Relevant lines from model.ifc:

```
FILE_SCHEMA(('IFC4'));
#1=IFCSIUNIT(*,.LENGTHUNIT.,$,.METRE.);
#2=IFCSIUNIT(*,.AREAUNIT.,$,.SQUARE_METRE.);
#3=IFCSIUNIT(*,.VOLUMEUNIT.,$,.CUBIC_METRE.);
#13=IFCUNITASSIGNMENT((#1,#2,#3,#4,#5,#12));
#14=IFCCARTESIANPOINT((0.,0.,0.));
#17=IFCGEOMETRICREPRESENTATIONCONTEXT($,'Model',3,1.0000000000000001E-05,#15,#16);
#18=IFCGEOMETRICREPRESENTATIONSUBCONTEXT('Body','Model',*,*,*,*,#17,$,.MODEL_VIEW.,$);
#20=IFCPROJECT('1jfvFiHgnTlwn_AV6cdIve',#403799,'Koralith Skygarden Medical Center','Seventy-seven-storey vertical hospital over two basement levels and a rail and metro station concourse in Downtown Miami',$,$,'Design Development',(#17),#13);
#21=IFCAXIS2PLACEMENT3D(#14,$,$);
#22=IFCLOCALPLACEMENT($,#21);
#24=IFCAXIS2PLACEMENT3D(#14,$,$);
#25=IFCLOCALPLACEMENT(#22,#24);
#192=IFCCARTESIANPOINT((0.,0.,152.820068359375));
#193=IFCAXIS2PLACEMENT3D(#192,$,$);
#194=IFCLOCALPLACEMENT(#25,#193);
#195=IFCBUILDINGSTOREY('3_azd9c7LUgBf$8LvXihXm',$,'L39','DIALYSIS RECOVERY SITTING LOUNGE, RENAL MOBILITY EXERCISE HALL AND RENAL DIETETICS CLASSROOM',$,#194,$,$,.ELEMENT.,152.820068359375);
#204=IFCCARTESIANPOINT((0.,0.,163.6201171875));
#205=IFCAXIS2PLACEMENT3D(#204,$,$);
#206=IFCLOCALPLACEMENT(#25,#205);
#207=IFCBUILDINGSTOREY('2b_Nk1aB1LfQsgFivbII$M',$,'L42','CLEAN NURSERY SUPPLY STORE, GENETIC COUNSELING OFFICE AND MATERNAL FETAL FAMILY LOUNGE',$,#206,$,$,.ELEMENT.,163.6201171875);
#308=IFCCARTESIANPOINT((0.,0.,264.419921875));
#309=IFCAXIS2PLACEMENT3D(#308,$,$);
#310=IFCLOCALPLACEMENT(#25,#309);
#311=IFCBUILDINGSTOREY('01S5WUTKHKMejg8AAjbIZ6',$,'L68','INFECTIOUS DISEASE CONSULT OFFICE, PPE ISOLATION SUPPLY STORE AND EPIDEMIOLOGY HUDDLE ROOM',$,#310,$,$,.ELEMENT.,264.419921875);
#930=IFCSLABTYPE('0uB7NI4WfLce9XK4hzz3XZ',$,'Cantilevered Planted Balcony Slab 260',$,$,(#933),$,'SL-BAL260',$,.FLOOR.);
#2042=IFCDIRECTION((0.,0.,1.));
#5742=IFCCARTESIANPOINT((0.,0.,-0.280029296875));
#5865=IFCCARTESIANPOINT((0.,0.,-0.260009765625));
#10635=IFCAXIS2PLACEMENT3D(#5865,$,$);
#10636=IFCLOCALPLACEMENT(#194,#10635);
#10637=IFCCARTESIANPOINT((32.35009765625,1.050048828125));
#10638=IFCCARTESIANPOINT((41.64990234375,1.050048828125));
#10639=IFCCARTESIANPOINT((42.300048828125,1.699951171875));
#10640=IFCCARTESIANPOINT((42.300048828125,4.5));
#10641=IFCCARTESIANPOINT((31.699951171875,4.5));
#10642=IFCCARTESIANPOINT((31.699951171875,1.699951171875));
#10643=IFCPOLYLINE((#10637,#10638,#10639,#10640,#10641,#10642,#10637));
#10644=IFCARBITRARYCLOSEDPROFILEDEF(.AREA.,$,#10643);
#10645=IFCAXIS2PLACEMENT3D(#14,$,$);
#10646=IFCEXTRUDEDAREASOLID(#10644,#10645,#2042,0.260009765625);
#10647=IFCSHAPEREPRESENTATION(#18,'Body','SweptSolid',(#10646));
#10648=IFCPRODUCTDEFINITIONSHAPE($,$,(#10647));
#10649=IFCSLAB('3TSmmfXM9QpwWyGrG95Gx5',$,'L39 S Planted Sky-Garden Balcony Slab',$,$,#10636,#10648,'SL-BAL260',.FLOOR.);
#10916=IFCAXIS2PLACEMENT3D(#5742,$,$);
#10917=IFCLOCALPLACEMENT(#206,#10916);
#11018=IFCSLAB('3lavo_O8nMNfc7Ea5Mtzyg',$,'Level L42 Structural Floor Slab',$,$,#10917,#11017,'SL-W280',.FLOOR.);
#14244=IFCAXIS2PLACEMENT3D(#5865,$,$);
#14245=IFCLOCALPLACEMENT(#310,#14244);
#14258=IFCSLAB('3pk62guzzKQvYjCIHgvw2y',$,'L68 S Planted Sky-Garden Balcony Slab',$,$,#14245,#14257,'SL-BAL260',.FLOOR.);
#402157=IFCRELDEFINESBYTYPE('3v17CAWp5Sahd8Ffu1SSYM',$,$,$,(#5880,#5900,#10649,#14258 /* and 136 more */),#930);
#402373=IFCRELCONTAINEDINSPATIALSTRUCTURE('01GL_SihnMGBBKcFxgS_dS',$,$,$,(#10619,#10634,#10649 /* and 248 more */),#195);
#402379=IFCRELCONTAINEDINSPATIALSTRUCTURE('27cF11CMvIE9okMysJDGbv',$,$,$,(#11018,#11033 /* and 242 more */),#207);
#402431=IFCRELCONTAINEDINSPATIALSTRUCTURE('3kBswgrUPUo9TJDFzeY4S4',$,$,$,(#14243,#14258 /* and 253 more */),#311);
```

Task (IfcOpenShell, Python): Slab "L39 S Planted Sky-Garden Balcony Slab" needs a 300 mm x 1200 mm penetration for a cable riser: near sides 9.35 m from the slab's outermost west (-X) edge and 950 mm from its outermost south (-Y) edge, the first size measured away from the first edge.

```python
import numpy as np
import ifcopenshell
import ifcopenshell.api.feature
import ifcopenshell.api.geometry
import ifcopenshell.api.root
import ifcopenshell.geom
import ifcopenshell.util.placement
import ifcopenshell.util.representation
import ifcopenshell.util.shape
import ifcopenshell.util.unit

model = ifcopenshell.open("model.ifc")
unit_scale = ifcopenshell.util.unit.calculate_unit_scale(model)
settings = ifcopenshell.geom.settings()


def volume(element):
    """Net volume in cubic metres, openings subtracted."""
    shape = ifcopenshell.geom.create_shape(settings, element)
    return ifcopenshell.util.shape.get_volume(shape.geometry)


slab = model.by_id(10649)
before = volume(slab)

# Extent in the slab's own axes, in metres. The edges named are its -X and -Y sides.
slab_shape = ifcopenshell.geom.create_shape(settings, slab)
vertices = ifcopenshell.util.shape.get_vertices(slab_shape.geometry)
x_min, y_min, bottom = vertices.min(axis=0)
top = vertices[:, 2].max()

opening = ifcopenshell.api.root.create_entity(model, ifc_class="IfcOpeningElement", name="Cable riser opening", predefined_type="OPENING")
context = ifcopenshell.util.representation.get_context(model, "Model", "Body", "MODEL_VIEW")
width, depth = 0.3, 1.2
outline = [(0.0, 0.0), (width, 0.0), (width, depth), (0.0, depth), (0.0, 0.0)]
# Overshoot both faces by 50 mm so the cut is clean.
shape = ifcopenshell.api.geometry.add_slab_representation(
    model, context=context, depth=top - bottom + 0.1, polyline=outline
)
ifcopenshell.api.geometry.assign_representation(model, product=opening, representation=shape)

matrix = ifcopenshell.util.placement.get_local_placement(slab.ObjectPlacement)
matrix[:, 3] = matrix @ np.append(np.array([x_min + 9.35, y_min + 0.95, bottom - 0.05]) / unit_scale, 1.0)
ifcopenshell.api.geometry.edit_object_placement(model, product=opening, matrix=matrix, is_si=False)
ifcopenshell.api.feature.add_feature(model, feature=opening, element=slab)

after = volume(slab)

print(f"slab volume {before:.3f} -> {after:.3f} m3")

model.write("model-out.ifc")
```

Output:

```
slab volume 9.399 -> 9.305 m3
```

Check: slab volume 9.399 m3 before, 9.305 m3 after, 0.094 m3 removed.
